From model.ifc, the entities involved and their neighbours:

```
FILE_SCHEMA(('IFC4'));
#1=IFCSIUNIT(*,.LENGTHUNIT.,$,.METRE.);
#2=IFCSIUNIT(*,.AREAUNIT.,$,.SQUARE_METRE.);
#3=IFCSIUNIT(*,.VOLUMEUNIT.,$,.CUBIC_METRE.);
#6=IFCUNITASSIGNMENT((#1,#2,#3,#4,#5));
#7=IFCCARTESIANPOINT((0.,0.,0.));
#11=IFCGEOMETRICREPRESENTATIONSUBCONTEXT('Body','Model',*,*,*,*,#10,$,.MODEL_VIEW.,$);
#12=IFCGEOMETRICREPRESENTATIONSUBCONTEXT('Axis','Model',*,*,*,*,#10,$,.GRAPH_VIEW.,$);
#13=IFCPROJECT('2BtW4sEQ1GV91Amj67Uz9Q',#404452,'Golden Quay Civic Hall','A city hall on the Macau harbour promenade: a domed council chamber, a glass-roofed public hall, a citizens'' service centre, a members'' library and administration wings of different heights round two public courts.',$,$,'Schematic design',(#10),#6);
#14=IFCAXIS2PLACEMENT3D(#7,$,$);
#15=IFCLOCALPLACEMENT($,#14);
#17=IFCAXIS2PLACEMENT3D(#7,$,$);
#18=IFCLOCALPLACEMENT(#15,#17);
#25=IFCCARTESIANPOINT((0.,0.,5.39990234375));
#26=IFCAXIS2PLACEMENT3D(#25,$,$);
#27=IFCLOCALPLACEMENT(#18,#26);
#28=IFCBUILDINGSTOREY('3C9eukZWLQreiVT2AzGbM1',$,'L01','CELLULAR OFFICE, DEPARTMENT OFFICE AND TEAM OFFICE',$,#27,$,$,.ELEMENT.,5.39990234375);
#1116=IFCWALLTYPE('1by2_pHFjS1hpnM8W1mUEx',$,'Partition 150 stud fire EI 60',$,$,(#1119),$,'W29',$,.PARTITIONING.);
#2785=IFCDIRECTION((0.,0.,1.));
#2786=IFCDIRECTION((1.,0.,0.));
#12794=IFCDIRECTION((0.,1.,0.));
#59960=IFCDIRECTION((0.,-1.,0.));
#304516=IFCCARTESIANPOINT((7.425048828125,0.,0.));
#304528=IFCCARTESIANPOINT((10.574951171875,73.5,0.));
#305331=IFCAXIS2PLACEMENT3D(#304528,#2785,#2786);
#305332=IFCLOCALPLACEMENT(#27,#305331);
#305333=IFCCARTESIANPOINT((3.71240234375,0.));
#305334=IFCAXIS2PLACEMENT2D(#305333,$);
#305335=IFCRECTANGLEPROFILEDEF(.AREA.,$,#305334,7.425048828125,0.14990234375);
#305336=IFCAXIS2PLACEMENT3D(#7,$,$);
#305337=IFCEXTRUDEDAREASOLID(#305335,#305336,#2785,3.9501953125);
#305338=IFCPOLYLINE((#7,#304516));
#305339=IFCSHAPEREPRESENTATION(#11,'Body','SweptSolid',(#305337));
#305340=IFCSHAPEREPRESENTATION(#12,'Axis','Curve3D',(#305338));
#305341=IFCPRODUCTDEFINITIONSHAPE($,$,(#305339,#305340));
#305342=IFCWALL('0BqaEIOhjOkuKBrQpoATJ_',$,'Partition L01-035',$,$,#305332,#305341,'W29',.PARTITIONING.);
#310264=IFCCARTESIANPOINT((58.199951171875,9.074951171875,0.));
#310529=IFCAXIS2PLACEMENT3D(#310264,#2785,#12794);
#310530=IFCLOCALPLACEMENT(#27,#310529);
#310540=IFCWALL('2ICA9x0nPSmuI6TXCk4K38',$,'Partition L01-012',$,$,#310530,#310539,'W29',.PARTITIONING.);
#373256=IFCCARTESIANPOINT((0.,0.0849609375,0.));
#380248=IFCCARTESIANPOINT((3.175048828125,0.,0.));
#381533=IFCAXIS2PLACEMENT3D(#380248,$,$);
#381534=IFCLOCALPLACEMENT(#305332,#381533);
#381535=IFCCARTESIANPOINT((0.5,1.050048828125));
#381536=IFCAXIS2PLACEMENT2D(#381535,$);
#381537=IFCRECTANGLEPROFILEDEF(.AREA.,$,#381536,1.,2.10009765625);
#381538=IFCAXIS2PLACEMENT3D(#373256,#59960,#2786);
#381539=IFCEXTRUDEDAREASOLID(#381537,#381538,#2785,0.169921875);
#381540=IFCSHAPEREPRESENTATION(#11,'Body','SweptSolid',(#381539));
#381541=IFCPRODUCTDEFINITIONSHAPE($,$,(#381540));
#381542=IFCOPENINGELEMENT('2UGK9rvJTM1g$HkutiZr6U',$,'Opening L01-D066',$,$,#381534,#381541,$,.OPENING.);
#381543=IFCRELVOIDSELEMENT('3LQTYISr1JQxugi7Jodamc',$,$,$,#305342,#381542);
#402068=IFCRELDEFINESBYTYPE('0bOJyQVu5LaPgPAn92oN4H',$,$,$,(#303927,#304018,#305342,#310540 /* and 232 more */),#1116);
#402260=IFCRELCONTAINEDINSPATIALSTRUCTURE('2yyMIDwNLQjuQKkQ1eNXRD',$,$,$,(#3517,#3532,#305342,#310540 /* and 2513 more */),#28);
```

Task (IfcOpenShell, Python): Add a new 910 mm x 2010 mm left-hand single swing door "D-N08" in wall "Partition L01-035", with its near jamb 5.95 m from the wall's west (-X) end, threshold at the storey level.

```python
import numpy as np
import ifcopenshell
import ifcopenshell.api.feature
import ifcopenshell.api.geometry
import ifcopenshell.api.root
import ifcopenshell.api.spatial
import ifcopenshell.geom
import ifcopenshell.util.element
import ifcopenshell.util.placement
import ifcopenshell.util.representation
import ifcopenshell.util.shape
import ifcopenshell.util.unit

model = ifcopenshell.open("model.ifc")
unit_scale = ifcopenshell.util.unit.calculate_unit_scale(model)
settings = ifcopenshell.geom.settings()


def volume(element):
    """Net volume in cubic metres, openings subtracted."""
    shape = ifcopenshell.geom.create_shape(settings, element)
    return ifcopenshell.util.shape.get_volume(shape.geometry)


wall = model.by_guid("0BqaEIOhjOkuKBrQpoATJ_")
storey = ifcopenshell.util.element.get_container(wall, ifc_class="IfcBuildingStorey")
context = ifcopenshell.util.representation.get_context(model, "Model", "Body", "MODEL_VIEW")
before = volume(wall)

width, height, from_end, sill = 0.91, 2.01, 5.95, 0.0  # metres

# The wall runs along its own X axis, and the end named is its -X end.
wall_shape = ifcopenshell.geom.create_shape(settings, wall)
x, y, z = ifcopenshell.util.shape.get_vertices(wall_shape.geometry).T
start = x.min() + from_end
face, thickness = float(y.min()), float(y.max() - y.min())
wall_matrix = ifcopenshell.util.placement.get_local_placement(wall.ObjectPlacement)
level = ifcopenshell.util.placement.get_local_placement(storey.ObjectPlacement)[2, 3]


def in_wall(x, y):
    """Placement at x, y metres in the wall's axes, at sill height."""
    matrix = wall_matrix.copy()
    matrix[:, 3] = wall_matrix @ np.array([x / unit_scale, y / unit_scale, 0.0, 1.0])
    matrix[2, 3] = level + sill / unit_scale
    return matrix


# Opening: a box that overshoots both wall faces by 50 mm.
opening = ifcopenshell.api.root.create_entity(model, ifc_class="IfcOpeningElement", predefined_type="OPENING")
box = ifcopenshell.api.geometry.add_wall_representation(
    model, context=context, length=width, height=height, thickness=thickness + 0.1
)
ifcopenshell.api.geometry.assign_representation(model, product=opening, representation=box)
ifcopenshell.api.geometry.edit_object_placement(model, product=opening, matrix=in_wall(start, face - 0.05), is_si=False)
ifcopenshell.api.feature.add_feature(model, feature=opening, element=wall)

door = ifcopenshell.api.root.create_entity(model, ifc_class="IfcDoor", name="D-N08", predefined_type="DOOR")
door.OverallWidth, door.OverallHeight = width / unit_scale, height / unit_scale
door.OperationType = "SINGLE_SWING_LEFT"
body = ifcopenshell.api.geometry.add_door_representation(
    model,
    context=context,
    overall_width=door.OverallWidth,
    overall_height=door.OverallHeight,
    operation_type="SINGLE_SWING_LEFT",
    lining_properties={"LiningDepth": thickness / unit_scale, "ThresholdDepth": thickness / unit_scale},
)
ifcopenshell.api.geometry.assign_representation(model, product=door, representation=body)
ifcopenshell.api.spatial.assign_container(model, products=[door], relating_structure=storey)
ifcopenshell.api.feature.add_filling(model, opening=opening, element=door)

# The lining spans the wall, so the door starts at the wall face.
ifcopenshell.api.geometry.edit_object_placement(model, product=door, matrix=in_wall(start, face), is_si=False)

after = volume(wall)

print(f"wall volume {before:.3f} -> {after:.3f} m3")

model.write("model_v2.ifc")
```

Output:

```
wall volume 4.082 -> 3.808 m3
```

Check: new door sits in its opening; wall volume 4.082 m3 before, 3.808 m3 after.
